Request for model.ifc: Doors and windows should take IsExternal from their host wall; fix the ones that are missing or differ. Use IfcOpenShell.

First a look at what the model holds.

```python
import ifcopenshell
import ifcopenshell.util.element

model = ifcopenshell.open("model.ifc")
print(model.schema)
seen = {}
for e in model.by_type("IfcDoor") + model.by_type("IfcWindow"):
    if not e.FillsVoids:
        continue
    host = e.FillsVoids[0].RelatingOpeningElement.VoidsElements[0].RelatingBuildingElement
    own = ifcopenshell.util.element.get_pset(e, f"Pset_{e.is_a()[3:].removesuffix('StandardCase')}Common", "IsExternal")
    wall = ifcopenshell.util.element.get_pset(host, "Pset_WallCommon", "IsExternal")
    seen[e.is_a(), own, wall] = seen.get((e.is_a(), own, wall), 0) + 1
for (cls, own, wall), count in sorted(seen.items(), key=str):
    print(count, cls, "IsExternal:", own, "| host wall:", wall)
```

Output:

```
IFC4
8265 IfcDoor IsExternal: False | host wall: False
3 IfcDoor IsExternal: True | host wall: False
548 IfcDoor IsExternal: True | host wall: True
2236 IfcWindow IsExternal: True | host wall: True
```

```python
import ifcopenshell
import ifcopenshell.api.pset
import ifcopenshell.util.element

model = ifcopenshell.open("model.ifc")

count = 0
for ifc_class, pset_name in (("IfcDoor", "Pset_DoorCommon"), ("IfcWindow", "Pset_WindowCommon")):
    for e in model.by_type(ifc_class):
        if not e.FillsVoids:
            continue
        host = e.FillsVoids[0].RelatingOpeningElement.VoidsElements[0].RelatingBuildingElement
        external = ifcopenshell.util.element.get_pset(host, "Pset_WallCommon", "IsExternal")
        if external is None or ifcopenshell.util.element.get_pset(e, pset_name, "IsExternal") == external:
            continue
        found = ifcopenshell.util.element.get_pset(e, pset_name, should_inherit=False)
        if found:
            pset = model.by_id(found["id"])
            if len(ifcopenshell.util.element.get_elements_by_pset(pset)) > 1:
                pset = ifcopenshell.api.pset.unshare_pset(model, products=[e], pset=pset)[0]
        else:
            pset = ifcopenshell.api.pset.add_pset(model, product=e, name=pset_name)
        ifcopenshell.api.pset.edit_pset(model, pset=pset, properties={"IsExternal": external})
        count += 1

print(count, "updated")

model.write("model_updated.ifc")
```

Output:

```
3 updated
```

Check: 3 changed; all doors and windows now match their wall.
